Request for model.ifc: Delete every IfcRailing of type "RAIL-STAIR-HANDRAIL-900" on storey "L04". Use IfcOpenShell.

First a look at what the model holds.

```python
import ifcopenshell
import ifcopenshell.util.element

model = ifcopenshell.open("model.ifc")
print(model.schema)
storey = next(s for s in model.by_type("IfcBuildingStorey") if s.Name == "L04")
railings = [e for e in ifcopenshell.util.element.get_decomposition(storey) if e.is_a("IfcRailing")]
seen = {}
for e in railings:
    element_type = ifcopenshell.util.element.get_type(e)
    name = element_type.Name if element_type not in (None, e) else None
    seen[name] = seen.get(name, 0) + 1
for name, count in sorted(seen.items(), key=str):
    print(count, "x", name)
```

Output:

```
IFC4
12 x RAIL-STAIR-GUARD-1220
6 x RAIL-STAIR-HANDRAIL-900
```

```python
import ifcopenshell
import ifcopenshell.api.root
import ifcopenshell.util.element

model = ifcopenshell.open("model.ifc")

storey = next(s for s in model.by_type("IfcBuildingStorey") if s.Name == "L04")
railings = [e for e in ifcopenshell.util.element.get_decomposition(storey) if e.is_a("IfcRailing")]
targets = [e for e in railings if (t := ifcopenshell.util.element.get_type(e)) not in (None, e) and t.Name == "RAIL-STAIR-HANDRAIL-900"]

for e in targets:
    ifcopenshell.api.root.remove_product(model, product=e)
print(len(targets), "removed")

model.write("model_rev.ifc")
```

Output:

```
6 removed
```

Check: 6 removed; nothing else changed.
